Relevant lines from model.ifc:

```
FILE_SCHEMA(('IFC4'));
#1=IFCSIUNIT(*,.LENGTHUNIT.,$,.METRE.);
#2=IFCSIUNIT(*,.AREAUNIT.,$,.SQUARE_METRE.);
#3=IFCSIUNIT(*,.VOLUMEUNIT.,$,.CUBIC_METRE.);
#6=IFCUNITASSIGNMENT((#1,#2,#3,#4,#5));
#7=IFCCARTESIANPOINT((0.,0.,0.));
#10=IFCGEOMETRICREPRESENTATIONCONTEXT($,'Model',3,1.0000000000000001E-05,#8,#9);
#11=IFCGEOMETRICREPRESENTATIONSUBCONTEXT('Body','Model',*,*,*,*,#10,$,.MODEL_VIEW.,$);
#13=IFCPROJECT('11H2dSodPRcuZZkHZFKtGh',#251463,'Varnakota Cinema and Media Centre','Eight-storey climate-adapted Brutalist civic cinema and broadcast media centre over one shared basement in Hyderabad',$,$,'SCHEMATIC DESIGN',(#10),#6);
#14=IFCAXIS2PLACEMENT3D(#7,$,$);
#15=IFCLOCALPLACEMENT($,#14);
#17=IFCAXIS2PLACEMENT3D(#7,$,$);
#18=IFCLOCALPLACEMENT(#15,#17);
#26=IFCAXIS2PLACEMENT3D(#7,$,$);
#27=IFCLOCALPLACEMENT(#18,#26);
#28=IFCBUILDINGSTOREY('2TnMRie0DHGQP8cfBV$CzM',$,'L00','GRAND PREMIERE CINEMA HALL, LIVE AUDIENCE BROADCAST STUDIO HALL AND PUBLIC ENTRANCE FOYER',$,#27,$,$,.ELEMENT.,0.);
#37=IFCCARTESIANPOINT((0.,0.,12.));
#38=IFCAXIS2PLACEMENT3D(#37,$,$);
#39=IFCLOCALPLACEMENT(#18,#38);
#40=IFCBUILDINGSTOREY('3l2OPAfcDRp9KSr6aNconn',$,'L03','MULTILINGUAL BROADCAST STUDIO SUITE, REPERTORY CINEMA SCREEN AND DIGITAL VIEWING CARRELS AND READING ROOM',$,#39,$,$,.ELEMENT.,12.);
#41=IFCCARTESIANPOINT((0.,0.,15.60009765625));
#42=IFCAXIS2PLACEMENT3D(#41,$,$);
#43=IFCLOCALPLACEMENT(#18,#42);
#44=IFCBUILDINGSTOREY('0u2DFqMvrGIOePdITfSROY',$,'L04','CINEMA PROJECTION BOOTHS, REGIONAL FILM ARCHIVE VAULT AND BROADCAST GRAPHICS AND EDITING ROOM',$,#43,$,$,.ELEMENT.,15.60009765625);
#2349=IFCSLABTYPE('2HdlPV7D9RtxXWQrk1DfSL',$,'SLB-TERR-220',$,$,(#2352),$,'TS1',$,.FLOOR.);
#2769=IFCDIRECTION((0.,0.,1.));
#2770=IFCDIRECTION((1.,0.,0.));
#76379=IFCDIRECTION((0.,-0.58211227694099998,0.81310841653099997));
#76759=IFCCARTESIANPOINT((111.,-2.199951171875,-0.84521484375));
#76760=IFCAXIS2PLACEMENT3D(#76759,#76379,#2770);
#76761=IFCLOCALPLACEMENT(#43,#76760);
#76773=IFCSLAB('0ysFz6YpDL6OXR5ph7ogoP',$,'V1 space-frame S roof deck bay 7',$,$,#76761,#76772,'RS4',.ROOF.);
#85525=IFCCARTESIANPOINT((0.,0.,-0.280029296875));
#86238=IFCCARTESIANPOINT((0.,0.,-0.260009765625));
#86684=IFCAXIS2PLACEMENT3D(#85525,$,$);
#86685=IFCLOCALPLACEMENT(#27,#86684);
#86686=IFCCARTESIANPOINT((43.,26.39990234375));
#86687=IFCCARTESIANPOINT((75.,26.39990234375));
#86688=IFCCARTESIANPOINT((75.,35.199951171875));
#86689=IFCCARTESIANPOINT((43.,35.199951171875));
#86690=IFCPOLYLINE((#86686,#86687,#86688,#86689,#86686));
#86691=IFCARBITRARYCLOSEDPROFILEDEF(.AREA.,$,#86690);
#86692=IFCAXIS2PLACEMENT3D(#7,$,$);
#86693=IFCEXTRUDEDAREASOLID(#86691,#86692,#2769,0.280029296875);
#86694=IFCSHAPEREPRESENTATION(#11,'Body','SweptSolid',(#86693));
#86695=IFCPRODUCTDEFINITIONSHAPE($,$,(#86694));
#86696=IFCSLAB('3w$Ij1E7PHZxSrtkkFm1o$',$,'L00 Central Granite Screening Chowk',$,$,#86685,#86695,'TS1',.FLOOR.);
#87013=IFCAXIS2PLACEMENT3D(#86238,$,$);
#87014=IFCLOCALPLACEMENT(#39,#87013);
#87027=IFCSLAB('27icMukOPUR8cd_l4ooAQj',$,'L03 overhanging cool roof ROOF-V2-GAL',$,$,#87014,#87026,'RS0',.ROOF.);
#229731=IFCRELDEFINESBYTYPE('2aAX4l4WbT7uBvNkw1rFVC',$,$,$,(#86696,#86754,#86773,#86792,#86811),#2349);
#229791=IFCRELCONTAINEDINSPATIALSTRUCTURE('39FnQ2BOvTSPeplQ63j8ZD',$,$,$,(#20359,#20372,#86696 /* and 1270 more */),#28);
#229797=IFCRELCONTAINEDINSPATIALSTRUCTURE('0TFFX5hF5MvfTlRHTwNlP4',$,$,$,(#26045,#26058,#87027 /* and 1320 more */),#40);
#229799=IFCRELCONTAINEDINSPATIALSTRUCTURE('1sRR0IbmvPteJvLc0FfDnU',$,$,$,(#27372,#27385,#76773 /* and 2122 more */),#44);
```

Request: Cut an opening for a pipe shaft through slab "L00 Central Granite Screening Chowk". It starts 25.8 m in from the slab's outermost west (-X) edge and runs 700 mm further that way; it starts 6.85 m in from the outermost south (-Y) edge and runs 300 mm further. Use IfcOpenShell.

```python
import numpy as np
import ifcopenshell
import ifcopenshell.api.feature
import ifcopenshell.api.geometry
import ifcopenshell.api.root
import ifcopenshell.geom
import ifcopenshell.util.placement
import ifcopenshell.util.representation
import ifcopenshell.util.shape
import ifcopenshell.util.unit

model = ifcopenshell.open("model.ifc")
unit_scale = ifcopenshell.util.unit.calculate_unit_scale(model)
settings = ifcopenshell.geom.settings()


def volume(element):
    """Net volume in cubic metres, openings subtracted."""
    shape = ifcopenshell.geom.create_shape(settings, element)
    return ifcopenshell.util.shape.get_volume(shape.geometry)


slab = model.by_id(86696)
before = volume(slab)

# Extent in the slab's own axes, in metres. The edges named are its -X and -Y sides.
slab_shape = ifcopenshell.geom.create_shape(settings, slab)
vertices = ifcopenshell.util.shape.get_vertices(slab_shape.geometry)
x_min, y_min, bottom = vertices.min(axis=0)
top = vertices[:, 2].max()

opening = ifcopenshell.api.root.create_entity(model, ifc_class="IfcOpeningElement", name="Pipe shaft opening", predefined_type="OPENING")
context = ifcopenshell.util.representation.get_context(model, "Model", "Body", "MODEL_VIEW")
width, depth = 0.7, 0.3
outline = [(0.0, 0.0), (width, 0.0), (width, depth), (0.0, depth), (0.0, 0.0)]
# Overshoot both faces by 50 mm so the cut is clean.
shape = ifcopenshell.api.geometry.add_slab_representation(
    model, context=context, depth=top - bottom + 0.1, polyline=outline
)
ifcopenshell.api.geometry.assign_representation(model, product=opening, representation=shape)

matrix = ifcopenshell.util.placement.get_local_placement(slab.ObjectPlacement)
matrix[:, 3] = matrix @ np.append(np.array([x_min + 25.8, y_min + 6.85, bottom - 0.05]) / unit_scale, 1.0)
ifcopenshell.api.geometry.edit_object_placement(model, product=opening, matrix=matrix, is_si=False)
ifcopenshell.api.feature.add_feature(model, feature=opening, element=slab)

after = volume(slab)

print(f"slab volume {before:.3f} -> {after:.3f} m3")

model.write("model_edited.ifc")
```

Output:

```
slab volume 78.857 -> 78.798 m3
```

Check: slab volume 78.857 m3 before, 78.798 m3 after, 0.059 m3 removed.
